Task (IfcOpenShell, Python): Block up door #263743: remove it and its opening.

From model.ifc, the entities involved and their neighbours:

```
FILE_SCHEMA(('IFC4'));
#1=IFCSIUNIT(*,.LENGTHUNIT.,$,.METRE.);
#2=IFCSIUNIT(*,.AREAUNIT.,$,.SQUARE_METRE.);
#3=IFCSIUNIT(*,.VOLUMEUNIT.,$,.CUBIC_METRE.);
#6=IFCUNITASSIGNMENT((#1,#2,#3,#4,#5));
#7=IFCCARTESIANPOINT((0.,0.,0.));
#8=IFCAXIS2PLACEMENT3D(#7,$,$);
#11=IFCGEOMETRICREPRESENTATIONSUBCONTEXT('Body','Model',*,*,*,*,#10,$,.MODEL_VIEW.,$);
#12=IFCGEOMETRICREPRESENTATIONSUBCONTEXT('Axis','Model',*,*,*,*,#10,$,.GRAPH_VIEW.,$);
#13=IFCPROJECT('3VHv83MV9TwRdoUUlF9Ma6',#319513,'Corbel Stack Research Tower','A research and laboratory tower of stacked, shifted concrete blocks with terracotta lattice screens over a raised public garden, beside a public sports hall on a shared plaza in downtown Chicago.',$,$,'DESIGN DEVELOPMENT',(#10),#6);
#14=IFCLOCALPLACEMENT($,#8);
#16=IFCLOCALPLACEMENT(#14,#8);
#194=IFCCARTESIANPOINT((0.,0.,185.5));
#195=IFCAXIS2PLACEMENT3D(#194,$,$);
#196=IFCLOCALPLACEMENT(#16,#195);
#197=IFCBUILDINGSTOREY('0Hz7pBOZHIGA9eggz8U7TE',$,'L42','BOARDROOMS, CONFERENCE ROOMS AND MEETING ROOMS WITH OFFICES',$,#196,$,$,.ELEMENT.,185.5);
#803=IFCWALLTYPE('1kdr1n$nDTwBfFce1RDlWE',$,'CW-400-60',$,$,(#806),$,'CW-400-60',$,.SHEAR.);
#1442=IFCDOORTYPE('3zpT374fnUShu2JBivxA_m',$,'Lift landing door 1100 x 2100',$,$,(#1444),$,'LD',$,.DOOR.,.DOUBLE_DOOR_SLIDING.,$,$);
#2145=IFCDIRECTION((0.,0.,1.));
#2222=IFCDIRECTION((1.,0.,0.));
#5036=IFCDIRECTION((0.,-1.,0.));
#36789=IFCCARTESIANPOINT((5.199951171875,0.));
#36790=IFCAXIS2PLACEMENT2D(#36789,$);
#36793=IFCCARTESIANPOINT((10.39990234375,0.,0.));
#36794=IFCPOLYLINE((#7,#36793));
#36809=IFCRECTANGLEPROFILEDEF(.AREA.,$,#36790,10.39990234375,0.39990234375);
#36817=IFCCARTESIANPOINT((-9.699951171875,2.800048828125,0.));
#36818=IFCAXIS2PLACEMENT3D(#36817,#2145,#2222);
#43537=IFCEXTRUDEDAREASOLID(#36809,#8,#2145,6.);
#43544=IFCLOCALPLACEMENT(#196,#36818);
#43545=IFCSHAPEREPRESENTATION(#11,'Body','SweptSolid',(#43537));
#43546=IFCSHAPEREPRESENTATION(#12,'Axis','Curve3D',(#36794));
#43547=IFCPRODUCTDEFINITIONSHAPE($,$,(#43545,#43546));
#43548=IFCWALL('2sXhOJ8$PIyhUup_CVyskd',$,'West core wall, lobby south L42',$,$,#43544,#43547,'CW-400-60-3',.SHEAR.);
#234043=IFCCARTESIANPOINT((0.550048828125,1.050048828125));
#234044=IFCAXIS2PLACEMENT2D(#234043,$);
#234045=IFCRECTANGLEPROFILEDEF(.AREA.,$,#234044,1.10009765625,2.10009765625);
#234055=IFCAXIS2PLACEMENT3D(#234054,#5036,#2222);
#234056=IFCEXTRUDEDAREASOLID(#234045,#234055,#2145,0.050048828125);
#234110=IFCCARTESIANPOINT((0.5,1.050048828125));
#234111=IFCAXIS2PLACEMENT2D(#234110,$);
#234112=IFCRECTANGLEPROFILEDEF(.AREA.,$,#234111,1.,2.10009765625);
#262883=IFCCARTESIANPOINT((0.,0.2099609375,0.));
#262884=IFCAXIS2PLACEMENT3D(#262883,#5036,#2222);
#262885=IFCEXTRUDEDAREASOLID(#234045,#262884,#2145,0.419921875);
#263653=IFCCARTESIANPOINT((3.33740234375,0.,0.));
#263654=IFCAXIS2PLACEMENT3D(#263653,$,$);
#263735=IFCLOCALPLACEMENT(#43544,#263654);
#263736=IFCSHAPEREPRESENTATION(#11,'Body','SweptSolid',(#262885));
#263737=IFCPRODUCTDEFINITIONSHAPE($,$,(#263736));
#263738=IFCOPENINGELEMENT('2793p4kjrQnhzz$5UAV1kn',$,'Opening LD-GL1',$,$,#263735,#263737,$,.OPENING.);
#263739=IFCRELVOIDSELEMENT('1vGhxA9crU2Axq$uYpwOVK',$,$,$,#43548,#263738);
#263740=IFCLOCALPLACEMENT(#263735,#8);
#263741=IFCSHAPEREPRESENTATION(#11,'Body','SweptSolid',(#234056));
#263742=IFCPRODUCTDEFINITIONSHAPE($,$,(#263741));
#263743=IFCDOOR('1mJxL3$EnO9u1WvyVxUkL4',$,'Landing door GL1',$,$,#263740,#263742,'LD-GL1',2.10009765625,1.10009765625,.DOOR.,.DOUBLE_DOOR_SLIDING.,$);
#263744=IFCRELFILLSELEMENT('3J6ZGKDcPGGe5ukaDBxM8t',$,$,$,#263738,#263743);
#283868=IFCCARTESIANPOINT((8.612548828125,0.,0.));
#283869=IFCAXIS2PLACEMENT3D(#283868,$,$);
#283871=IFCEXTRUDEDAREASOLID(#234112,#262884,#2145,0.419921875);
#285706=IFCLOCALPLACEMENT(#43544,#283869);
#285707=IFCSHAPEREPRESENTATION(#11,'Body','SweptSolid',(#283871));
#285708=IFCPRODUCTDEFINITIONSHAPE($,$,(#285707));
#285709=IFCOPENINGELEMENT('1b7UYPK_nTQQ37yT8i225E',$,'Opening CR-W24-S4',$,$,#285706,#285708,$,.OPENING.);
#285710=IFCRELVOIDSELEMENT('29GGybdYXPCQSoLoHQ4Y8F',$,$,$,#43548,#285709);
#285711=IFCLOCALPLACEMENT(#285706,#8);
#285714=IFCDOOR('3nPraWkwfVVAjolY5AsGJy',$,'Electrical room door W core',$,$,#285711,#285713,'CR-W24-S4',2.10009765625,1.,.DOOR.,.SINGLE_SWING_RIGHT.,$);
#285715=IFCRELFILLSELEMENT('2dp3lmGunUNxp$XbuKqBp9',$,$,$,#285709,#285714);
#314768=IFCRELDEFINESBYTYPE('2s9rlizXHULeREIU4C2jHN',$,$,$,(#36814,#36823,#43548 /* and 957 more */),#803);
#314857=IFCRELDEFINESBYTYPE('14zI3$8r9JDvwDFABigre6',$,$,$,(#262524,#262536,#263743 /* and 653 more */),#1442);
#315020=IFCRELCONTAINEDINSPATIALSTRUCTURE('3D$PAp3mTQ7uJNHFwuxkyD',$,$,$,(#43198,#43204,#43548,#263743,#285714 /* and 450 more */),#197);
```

```python
import ifcopenshell
import ifcopenshell.api.feature
import ifcopenshell.api.root
import ifcopenshell.geom
import ifcopenshell.util.shape

model = ifcopenshell.open("model.ifc")
settings = ifcopenshell.geom.settings()


def volume(element):
    """Net volume in cubic metres, openings subtracted."""
    shape = ifcopenshell.geom.create_shape(settings, element)
    return ifcopenshell.util.shape.get_volume(shape.geometry)


door = model.by_id(263743)
opening = door.FillsVoids[0].RelatingOpeningElement
wall = opening.VoidsElements[0].RelatingBuildingElement
before = volume(wall)

ifcopenshell.api.root.remove_product(model, product=door)
ifcopenshell.api.feature.remove_feature(model, feature=opening)

after = volume(wall)

print(f"wall volume {before:.3f} -> {after:.3f} m3")

model.write("model_edited.ifc")
```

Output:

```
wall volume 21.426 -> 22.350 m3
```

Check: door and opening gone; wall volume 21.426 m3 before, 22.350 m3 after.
